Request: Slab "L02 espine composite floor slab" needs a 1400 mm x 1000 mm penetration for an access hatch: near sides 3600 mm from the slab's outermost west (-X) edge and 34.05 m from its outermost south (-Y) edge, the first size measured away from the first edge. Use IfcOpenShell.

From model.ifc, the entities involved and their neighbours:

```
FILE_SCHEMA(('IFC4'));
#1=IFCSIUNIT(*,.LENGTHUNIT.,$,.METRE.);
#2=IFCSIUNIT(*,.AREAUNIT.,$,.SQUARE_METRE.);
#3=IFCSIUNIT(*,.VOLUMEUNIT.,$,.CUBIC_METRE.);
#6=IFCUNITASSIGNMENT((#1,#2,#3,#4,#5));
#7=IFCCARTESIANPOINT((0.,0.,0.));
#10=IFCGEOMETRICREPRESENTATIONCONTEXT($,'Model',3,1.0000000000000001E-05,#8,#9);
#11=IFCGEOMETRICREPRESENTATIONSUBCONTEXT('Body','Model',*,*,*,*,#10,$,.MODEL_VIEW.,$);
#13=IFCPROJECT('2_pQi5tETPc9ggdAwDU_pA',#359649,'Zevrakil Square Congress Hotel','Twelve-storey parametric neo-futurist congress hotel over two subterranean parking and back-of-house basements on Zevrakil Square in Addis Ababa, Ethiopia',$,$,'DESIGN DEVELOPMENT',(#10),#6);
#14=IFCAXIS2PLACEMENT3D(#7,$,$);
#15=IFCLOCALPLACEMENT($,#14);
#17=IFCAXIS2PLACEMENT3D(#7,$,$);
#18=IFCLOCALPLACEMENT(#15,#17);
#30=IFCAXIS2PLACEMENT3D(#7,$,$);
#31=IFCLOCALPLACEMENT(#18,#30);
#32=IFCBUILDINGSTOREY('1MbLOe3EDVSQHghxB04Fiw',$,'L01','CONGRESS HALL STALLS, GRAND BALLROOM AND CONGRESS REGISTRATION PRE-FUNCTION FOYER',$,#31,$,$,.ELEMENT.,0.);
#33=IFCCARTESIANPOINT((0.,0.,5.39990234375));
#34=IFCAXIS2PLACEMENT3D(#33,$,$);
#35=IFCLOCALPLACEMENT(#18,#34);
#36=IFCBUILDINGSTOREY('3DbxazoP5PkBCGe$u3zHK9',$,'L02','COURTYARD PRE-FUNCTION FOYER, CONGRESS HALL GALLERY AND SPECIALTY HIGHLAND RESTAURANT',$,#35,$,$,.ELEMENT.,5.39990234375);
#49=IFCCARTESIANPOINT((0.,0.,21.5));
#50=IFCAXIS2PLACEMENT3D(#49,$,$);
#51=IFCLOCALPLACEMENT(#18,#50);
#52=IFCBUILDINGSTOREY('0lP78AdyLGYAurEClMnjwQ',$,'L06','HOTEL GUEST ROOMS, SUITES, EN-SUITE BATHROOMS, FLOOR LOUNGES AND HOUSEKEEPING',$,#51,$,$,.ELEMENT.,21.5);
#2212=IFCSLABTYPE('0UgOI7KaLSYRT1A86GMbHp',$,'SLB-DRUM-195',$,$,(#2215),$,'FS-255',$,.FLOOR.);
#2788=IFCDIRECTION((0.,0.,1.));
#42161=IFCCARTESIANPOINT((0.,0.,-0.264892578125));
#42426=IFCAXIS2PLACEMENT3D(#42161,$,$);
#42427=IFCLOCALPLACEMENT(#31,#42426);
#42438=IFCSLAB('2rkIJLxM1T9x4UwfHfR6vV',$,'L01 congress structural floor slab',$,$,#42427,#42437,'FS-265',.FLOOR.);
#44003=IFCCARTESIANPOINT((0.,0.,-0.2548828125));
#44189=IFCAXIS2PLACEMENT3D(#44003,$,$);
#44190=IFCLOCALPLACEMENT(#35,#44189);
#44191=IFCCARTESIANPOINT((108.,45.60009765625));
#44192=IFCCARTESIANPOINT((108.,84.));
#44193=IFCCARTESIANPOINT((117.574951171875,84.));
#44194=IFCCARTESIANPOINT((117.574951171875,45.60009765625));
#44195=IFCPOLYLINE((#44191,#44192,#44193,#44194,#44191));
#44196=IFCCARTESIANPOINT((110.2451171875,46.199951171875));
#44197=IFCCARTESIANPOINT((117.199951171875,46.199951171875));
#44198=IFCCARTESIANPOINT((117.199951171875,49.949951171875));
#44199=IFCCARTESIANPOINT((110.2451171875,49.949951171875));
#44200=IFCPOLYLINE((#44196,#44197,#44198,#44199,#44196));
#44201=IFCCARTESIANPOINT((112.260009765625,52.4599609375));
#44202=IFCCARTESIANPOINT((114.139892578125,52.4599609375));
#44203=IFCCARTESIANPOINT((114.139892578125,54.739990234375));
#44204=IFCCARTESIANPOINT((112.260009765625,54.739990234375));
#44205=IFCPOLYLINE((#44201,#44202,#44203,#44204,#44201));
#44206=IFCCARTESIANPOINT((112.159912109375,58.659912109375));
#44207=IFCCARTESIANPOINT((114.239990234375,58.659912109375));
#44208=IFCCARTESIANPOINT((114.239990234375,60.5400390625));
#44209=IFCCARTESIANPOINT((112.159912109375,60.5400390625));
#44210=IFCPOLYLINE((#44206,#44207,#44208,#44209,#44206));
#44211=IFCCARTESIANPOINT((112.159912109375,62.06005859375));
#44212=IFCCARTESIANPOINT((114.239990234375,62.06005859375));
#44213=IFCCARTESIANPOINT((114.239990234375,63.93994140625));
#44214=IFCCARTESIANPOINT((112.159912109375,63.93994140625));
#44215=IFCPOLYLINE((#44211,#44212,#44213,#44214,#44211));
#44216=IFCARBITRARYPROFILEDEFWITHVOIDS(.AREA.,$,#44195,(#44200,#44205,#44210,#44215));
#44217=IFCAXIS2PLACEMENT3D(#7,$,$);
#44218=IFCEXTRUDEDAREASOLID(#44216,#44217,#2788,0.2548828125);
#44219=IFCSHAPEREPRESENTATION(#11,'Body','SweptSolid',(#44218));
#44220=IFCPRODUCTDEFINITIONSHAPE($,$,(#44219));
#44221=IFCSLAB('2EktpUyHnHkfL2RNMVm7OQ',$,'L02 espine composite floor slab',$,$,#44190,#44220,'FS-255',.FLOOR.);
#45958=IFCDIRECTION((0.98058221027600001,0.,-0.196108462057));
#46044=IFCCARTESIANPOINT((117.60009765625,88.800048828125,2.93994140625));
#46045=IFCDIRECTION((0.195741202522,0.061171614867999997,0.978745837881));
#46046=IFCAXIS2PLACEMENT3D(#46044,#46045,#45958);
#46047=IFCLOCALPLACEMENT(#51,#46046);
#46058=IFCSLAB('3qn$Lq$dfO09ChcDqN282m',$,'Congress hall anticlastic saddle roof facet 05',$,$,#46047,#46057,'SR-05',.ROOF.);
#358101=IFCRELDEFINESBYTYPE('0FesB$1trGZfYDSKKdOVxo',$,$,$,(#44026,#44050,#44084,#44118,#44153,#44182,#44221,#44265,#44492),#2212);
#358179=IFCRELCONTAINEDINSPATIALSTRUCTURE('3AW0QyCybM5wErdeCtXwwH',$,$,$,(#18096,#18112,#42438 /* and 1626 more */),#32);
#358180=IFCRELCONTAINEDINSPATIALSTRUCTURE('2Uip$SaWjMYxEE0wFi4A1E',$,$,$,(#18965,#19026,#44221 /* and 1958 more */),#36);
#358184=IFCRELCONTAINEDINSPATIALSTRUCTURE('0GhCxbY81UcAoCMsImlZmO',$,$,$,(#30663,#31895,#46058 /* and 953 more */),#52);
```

```python
import numpy as np
import ifcopenshell
import ifcopenshell.api.feature
import ifcopenshell.api.geometry
import ifcopenshell.api.root
import ifcopenshell.geom
import ifcopenshell.util.placement
import ifcopenshell.util.representation
import ifcopenshell.util.shape
import ifcopenshell.util.unit

model = ifcopenshell.open("model.ifc")
unit_scale = ifcopenshell.util.unit.calculate_unit_scale(model)
settings = ifcopenshell.geom.settings()


def volume(element):
    """Net volume in cubic metres, openings subtracted."""
    shape = ifcopenshell.geom.create_shape(settings, element)
    return ifcopenshell.util.shape.get_volume(shape.geometry)


slab = model.by_guid("2EktpUyHnHkfL2RNMVm7OQ")
before = volume(slab)

# Extent in the slab's own axes, in metres. The edges named are its -X and -Y sides.
slab_shape = ifcopenshell.geom.create_shape(settings, slab)
vertices = ifcopenshell.util.shape.get_vertices(slab_shape.geometry)
x_min, y_min, bottom = vertices.min(axis=0)
top = vertices[:, 2].max()

opening = ifcopenshell.api.root.create_entity(model, ifc_class="IfcOpeningElement", name="Access hatch opening", predefined_type="OPENING")
context = ifcopenshell.util.representation.get_context(model, "Model", "Body", "MODEL_VIEW")
width, depth = 1.4, 1
outline = [(0.0, 0.0), (width, 0.0), (width, depth), (0.0, depth), (0.0, 0.0)]
# Overshoot both faces by 50 mm so the cut is clean.
shape = ifcopenshell.api.geometry.add_slab_representation(
    model, context=context, depth=top - bottom + 0.1, polyline=outline
)
ifcopenshell.api.geometry.assign_representation(model, product=opening, representation=shape)

matrix = ifcopenshell.util.placement.get_local_placement(slab.ObjectPlacement)
matrix[:, 3] = matrix @ np.append(np.array([x_min + 3.6, y_min + 34.05, bottom - 0.05]) / unit_scale, 1.0)
ifcopenshell.api.geometry.edit_object_placement(model, product=opening, matrix=matrix, is_si=False)
ifcopenshell.api.feature.add_feature(model, feature=opening, element=slab)

after = volume(slab)

print(f"slab volume {before:.3f} -> {after:.3f} m3")

model.write("model-out.ifc")
```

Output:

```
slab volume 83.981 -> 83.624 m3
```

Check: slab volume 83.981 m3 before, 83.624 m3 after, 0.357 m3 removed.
